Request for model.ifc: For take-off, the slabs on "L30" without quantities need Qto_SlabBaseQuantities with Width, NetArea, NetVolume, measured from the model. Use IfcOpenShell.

First a look at what the model holds.

```python
import ifcopenshell
import ifcopenshell.util.element
import ifcopenshell.util.unit

model = ifcopenshell.open("model.ifc")
print(model.schema)
for unit_type in ("LENGTHUNIT", "AREAUNIT", "VOLUMEUNIT"):
    print(unit_type, ifcopenshell.util.unit.calculate_unit_scale(model, unit_type))
storey = next(s for s in model.by_type("IfcBuildingStorey") if s.Name == "L30")
slabs = [e for e in ifcopenshell.util.element.get_decomposition(storey) if e.is_a("IfcSlab")]
for e in sorted(slabs, key=lambda e: e.id()):
    print(e.id(), e.is_a(), e.Name, list(ifcopenshell.util.element.get_psets(e, qtos_only=True)), sep=" | ")
```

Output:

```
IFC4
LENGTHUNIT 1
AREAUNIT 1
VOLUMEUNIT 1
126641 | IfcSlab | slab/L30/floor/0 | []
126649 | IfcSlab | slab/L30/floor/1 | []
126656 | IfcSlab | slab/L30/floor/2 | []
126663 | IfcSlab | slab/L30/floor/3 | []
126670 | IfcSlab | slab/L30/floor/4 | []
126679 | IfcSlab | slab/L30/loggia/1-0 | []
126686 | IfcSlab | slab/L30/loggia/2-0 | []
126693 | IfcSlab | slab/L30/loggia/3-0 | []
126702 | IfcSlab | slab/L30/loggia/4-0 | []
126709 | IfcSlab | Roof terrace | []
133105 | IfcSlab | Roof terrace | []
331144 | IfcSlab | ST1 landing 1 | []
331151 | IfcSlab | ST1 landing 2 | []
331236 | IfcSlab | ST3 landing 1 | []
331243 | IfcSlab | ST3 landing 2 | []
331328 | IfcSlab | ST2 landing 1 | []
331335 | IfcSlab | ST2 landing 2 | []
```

```python
import ifcopenshell
import ifcopenshell.api.pset
import ifcopenshell.geom
import ifcopenshell.util.element
import ifcopenshell.util.shape
import ifcopenshell.util.unit

model = ifcopenshell.open("model.ifc")
unit_scale = ifcopenshell.util.unit.calculate_unit_scale(model)
area_scale = ifcopenshell.util.unit.calculate_unit_scale(model, "AREAUNIT")
volume_scale = ifcopenshell.util.unit.calculate_unit_scale(model, "VOLUMEUNIT")
settings = ifcopenshell.geom.settings()

storey = next(s for s in model.by_type("IfcBuildingStorey") if s.Name == "L30")
slabs = [e for e in ifcopenshell.util.element.get_decomposition(storey) if e.is_a("IfcSlab")]

for e in sorted(slabs, key=lambda e: e.id()):
    if ifcopenshell.util.element.get_psets(e, qtos_only=True, should_inherit=False):
        continue
    # Geometry comes back in metres, in the element's own axes.
    shape = ifcopenshell.geom.create_shape(settings, e)
    values = {
        "Width": ifcopenshell.util.shape.get_z(shape.geometry) / unit_scale,
        "NetArea": ifcopenshell.util.shape.get_footprint_area(shape.geometry) / area_scale,
        "NetVolume": ifcopenshell.util.shape.get_volume(shape.geometry) / volume_scale,
    }
    qto = ifcopenshell.api.pset.add_qto(model, product=e, name="Qto_SlabBaseQuantities")
    ifcopenshell.api.pset.edit_qto(model, qto=qto, properties=values)
    print(e.id(), {k: round(v, 3) for k, v in values.items()})

model.write("model_rev.ifc")
```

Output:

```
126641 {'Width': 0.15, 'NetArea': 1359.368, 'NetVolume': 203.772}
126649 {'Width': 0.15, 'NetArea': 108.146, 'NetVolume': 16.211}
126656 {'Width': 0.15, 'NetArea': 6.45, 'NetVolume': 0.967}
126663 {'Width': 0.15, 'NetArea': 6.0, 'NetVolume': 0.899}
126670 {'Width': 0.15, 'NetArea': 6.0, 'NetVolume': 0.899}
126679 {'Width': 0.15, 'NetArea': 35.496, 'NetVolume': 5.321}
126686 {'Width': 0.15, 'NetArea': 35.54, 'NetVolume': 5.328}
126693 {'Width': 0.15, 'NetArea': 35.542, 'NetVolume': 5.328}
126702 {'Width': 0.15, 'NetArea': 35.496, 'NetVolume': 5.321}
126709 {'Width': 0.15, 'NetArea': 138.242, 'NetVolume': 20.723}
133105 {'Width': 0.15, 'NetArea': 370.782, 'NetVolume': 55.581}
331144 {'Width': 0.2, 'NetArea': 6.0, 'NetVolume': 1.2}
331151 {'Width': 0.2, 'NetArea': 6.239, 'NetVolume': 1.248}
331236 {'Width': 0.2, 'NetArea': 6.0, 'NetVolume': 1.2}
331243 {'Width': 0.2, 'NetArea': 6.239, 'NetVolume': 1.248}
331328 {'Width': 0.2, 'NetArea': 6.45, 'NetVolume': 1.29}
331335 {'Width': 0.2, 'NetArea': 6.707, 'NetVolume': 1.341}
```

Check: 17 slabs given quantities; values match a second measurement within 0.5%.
